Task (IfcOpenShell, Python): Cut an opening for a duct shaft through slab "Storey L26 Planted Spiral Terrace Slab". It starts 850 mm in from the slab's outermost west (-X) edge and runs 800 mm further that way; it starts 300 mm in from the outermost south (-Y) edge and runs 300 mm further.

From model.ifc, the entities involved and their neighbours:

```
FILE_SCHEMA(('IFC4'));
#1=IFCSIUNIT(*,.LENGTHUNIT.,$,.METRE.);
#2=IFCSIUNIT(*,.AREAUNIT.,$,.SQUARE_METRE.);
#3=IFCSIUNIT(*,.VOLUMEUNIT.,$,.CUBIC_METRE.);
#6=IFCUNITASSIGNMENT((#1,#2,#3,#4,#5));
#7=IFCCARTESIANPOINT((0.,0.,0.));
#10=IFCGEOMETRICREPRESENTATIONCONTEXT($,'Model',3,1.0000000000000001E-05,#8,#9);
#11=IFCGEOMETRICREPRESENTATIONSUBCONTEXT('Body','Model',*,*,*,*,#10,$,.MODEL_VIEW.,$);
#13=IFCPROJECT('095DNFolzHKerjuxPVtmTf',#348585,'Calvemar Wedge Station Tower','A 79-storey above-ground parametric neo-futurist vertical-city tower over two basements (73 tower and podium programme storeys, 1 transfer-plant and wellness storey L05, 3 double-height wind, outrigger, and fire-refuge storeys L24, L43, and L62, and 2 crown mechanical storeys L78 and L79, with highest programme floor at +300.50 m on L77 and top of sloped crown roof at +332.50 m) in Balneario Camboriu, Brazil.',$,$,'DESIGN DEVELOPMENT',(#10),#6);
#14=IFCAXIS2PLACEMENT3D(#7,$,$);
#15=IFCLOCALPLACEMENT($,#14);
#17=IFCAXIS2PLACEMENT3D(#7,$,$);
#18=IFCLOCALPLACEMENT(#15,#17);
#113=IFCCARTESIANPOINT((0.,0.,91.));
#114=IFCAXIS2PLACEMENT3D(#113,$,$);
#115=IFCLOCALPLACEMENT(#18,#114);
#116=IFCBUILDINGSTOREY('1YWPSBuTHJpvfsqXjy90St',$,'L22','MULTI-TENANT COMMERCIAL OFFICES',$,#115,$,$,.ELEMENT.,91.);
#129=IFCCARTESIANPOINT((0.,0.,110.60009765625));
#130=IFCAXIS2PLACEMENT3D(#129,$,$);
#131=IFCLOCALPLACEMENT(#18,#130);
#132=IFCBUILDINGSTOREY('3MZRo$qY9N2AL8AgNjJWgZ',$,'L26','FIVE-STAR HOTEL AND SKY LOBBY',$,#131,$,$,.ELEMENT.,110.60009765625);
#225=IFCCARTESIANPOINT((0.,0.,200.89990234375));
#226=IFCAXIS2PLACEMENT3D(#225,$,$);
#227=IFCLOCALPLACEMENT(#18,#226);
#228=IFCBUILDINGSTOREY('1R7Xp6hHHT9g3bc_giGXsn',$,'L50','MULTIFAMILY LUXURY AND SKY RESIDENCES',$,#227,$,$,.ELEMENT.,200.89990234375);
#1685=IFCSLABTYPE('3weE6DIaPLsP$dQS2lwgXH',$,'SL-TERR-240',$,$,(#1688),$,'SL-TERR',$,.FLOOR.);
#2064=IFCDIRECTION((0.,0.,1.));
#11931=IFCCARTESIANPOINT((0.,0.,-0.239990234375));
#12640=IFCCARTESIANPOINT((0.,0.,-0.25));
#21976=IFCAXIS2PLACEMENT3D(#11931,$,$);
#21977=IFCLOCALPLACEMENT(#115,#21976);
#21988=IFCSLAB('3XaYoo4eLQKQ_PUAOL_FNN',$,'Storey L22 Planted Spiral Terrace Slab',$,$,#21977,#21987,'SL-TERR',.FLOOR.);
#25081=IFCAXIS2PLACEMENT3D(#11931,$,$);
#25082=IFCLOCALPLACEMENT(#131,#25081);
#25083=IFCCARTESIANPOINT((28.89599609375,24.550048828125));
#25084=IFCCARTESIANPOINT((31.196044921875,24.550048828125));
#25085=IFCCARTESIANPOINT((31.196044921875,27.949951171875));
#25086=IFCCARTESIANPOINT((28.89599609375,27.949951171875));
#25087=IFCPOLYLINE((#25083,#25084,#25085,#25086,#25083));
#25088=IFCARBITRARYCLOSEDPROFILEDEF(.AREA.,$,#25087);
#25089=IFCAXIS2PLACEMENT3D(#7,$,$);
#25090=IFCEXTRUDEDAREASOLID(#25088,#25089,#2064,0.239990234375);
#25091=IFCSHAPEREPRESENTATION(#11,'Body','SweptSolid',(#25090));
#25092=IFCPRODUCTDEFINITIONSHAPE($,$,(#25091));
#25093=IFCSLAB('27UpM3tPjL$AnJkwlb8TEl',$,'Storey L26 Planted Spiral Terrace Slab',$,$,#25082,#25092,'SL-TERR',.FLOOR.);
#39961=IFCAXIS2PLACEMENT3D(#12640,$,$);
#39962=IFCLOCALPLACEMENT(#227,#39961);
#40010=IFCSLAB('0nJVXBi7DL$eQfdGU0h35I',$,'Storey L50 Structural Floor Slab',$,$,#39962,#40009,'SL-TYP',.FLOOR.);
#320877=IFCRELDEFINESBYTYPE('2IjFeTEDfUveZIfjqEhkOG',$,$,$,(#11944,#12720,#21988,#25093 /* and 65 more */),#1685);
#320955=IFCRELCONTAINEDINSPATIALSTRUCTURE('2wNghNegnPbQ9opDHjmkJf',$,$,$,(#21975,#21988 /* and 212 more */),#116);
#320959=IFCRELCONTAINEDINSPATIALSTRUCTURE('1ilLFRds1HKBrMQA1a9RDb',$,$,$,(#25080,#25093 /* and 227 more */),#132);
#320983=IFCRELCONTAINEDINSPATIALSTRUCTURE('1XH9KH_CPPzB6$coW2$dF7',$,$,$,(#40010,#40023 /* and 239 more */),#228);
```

```python
import numpy as np
import ifcopenshell
import ifcopenshell.api.feature
import ifcopenshell.api.geometry
import ifcopenshell.api.root
import ifcopenshell.geom
import ifcopenshell.util.placement
import ifcopenshell.util.representation
import ifcopenshell.util.shape
import ifcopenshell.util.unit

model = ifcopenshell.open("model.ifc")
unit_scale = ifcopenshell.util.unit.calculate_unit_scale(model)
settings = ifcopenshell.geom.settings()


def volume(element):
    """Net volume in cubic metres, openings subtracted."""
    shape = ifcopenshell.geom.create_shape(settings, element)
    return ifcopenshell.util.shape.get_volume(shape.geometry)


slab = model.by_guid("27UpM3tPjL$AnJkwlb8TEl")
before = volume(slab)

# Extent in the slab's own axes, in metres. The edges named are its -X and -Y sides.
slab_shape = ifcopenshell.geom.create_shape(settings, slab)
vertices = ifcopenshell.util.shape.get_vertices(slab_shape.geometry)
x_min, y_min, bottom = vertices.min(axis=0)
top = vertices[:, 2].max()

opening = ifcopenshell.api.root.create_entity(model, ifc_class="IfcOpeningElement", name="Duct shaft opening", predefined_type="OPENING")
context = ifcopenshell.util.representation.get_context(model, "Model", "Body", "MODEL_VIEW")
width, depth = 0.8, 0.3
outline = [(0.0, 0.0), (width, 0.0), (width, depth), (0.0, depth), (0.0, 0.0)]
# Overshoot both faces by 50 mm so the cut is clean.
shape = ifcopenshell.api.geometry.add_slab_representation(
    model, context=context, depth=top - bottom + 0.1, polyline=outline
)
ifcopenshell.api.geometry.assign_representation(model, product=opening, representation=shape)

matrix = ifcopenshell.util.placement.get_local_placement(slab.ObjectPlacement)
matrix[:, 3] = matrix @ np.append(np.array([x_min + 0.85, y_min + 0.3, bottom - 0.05]) / unit_scale, 1.0)
ifcopenshell.api.geometry.edit_object_placement(model, product=opening, matrix=matrix, is_si=False)
ifcopenshell.api.feature.add_feature(model, feature=opening, element=slab)

after = volume(slab)

print(f"slab volume {before:.3f} -> {after:.3f} m3")

model.write("model_rev.ifc")
```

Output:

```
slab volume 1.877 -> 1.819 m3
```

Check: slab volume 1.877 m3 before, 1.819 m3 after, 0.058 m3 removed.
